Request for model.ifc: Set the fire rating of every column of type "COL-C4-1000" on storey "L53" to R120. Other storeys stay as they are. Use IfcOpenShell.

First a look at what the model holds.

```python
import ifcopenshell
import ifcopenshell.util.element

model = ifcopenshell.open("model.ifc")
print(model.schema)
storey = next(s for s in model.by_type("IfcBuildingStorey") if s.Name == "L53")
columns = [e for e in ifcopenshell.util.element.get_decomposition(storey) if e.is_a("IfcColumn")]
seen = {}
for e in columns:
    element_type = ifcopenshell.util.element.get_type(e)
    key = (element_type.Name if element_type != e and element_type else None, ifcopenshell.util.element.get_pset(e, "Pset_ColumnCommon", "FireRating"))
    seen[key] = seen.get(key, 0) + 1
for (name, value), count in sorted(seen.items(), key=str):
    print(count, "x", name, "|", value)
```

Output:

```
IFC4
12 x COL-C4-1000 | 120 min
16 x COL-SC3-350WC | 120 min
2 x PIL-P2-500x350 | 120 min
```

```python
import ifcopenshell
import ifcopenshell.api.pset
import ifcopenshell.util.element

model = ifcopenshell.open("model.ifc")

storey = next(s for s in model.by_type("IfcBuildingStorey") if s.Name == "L53")
columns = [e for e in ifcopenshell.util.element.get_decomposition(storey) if e.is_a("IfcColumn")]

count = 0
for e in columns:
    element_type = ifcopenshell.util.element.get_type(e)
    if element_type in (None, e) or element_type.Name != "COL-C4-1000":
        continue
    # add_pset returns the element's existing set when there is one.
    pset = ifcopenshell.api.pset.add_pset(model, product=e, name="Pset_ColumnCommon")
    ifcopenshell.api.pset.edit_pset(model, pset=pset, properties={"FireRating": "R120"})
    count += 1

print(count, "columns updated")

model.write("model_edited.ifc")
```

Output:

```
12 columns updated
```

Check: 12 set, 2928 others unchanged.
